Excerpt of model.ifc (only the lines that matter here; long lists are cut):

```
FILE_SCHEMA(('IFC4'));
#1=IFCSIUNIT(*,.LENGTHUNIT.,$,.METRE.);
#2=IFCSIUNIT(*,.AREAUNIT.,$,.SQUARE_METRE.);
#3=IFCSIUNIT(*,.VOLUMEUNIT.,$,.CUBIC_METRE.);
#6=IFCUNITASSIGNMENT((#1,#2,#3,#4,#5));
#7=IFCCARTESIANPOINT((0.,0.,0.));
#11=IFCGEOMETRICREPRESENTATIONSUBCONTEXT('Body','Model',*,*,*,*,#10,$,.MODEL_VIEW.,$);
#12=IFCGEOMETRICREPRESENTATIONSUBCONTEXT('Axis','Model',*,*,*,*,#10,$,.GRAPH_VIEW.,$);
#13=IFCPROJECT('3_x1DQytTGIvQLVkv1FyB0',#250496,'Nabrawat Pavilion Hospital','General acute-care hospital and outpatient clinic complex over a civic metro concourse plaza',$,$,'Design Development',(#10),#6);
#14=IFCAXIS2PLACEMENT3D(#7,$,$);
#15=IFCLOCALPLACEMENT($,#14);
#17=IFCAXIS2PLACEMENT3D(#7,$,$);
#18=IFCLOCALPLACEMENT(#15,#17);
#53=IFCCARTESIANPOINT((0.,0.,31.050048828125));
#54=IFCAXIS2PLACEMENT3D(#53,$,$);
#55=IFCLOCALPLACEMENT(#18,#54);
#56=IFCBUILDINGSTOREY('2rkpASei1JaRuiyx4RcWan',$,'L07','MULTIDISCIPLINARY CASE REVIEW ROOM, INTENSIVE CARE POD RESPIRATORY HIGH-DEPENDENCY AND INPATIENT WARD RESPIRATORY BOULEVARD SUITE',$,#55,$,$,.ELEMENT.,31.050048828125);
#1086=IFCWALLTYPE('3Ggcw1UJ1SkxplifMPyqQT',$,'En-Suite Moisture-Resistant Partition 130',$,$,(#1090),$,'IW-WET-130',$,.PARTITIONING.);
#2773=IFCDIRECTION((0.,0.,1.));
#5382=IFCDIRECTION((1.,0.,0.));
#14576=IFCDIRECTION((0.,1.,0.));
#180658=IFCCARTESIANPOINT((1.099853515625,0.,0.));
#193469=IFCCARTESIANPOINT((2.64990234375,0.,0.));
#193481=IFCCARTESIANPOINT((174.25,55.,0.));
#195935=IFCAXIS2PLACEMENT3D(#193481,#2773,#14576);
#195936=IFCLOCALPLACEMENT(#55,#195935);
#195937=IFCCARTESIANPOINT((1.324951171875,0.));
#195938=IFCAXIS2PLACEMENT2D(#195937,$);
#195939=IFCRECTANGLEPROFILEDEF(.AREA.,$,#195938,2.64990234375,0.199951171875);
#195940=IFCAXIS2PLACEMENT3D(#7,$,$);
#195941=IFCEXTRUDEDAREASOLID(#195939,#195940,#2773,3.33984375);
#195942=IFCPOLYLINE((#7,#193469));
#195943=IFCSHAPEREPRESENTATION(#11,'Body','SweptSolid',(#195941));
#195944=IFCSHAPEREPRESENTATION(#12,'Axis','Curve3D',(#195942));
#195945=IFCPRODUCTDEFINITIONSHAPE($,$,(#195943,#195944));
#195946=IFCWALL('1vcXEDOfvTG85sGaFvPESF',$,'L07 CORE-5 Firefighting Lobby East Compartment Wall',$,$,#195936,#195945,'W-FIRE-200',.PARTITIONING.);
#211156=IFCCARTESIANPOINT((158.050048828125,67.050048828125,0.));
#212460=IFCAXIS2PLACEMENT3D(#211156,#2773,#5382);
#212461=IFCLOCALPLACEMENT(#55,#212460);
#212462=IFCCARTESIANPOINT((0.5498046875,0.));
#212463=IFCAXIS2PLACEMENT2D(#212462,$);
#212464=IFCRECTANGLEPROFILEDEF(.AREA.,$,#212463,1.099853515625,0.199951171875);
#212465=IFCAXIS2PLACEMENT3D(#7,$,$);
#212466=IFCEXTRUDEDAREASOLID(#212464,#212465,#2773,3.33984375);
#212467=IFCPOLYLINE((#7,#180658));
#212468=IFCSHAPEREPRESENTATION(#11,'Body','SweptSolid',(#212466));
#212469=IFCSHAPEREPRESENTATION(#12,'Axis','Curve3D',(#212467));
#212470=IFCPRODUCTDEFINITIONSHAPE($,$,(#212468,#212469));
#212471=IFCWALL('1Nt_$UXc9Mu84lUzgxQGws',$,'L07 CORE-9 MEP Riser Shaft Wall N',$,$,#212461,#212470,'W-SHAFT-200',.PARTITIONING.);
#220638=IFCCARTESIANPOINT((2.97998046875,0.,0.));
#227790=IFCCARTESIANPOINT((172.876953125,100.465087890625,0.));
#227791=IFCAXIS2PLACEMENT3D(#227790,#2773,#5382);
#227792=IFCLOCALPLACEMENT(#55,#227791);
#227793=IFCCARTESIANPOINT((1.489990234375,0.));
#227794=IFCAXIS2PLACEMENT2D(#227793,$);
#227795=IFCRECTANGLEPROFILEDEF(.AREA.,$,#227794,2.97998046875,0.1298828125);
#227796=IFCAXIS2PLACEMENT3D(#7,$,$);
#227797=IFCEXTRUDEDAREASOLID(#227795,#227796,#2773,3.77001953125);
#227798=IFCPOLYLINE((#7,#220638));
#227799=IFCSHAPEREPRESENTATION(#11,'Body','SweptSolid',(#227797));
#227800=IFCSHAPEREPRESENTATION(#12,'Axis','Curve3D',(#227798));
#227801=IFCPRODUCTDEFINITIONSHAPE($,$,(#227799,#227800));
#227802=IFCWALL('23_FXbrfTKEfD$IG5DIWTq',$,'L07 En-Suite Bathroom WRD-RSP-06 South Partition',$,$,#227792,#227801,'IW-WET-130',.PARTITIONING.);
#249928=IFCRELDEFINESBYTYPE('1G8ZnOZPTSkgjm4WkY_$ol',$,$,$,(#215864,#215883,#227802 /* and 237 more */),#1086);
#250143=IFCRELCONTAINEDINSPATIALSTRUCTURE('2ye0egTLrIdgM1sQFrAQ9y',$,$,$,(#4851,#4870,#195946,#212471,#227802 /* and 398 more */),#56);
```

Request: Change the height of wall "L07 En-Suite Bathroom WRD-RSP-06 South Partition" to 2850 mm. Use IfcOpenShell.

```python
import ifcopenshell
import ifcopenshell.geom
import ifcopenshell.util.representation
import ifcopenshell.util.shape

model = ifcopenshell.open("model.ifc")
settings = ifcopenshell.geom.settings()


def volume(element):
    """Net volume in cubic metres, openings subtracted."""
    shape = ifcopenshell.geom.create_shape(settings, element)
    return ifcopenshell.util.shape.get_volume(shape.geometry)


wall = model.by_guid("23_FXbrfTKEfD$IG5DIWTq")
before = volume(wall)

body = ifcopenshell.util.representation.get_representation(wall, "Model", "Body")
solid = body.Items[0]
old_height = solid.Depth
solid.Depth = 2.85
after = volume(wall)

print(f"height {old_height:g} -> {solid.Depth:g}, volume {before:.3f} -> {after:.3f} m3")

model.write("model_rev.ifc")
```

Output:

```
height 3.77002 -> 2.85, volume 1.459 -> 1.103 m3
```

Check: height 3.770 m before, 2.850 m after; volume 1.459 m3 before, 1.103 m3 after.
